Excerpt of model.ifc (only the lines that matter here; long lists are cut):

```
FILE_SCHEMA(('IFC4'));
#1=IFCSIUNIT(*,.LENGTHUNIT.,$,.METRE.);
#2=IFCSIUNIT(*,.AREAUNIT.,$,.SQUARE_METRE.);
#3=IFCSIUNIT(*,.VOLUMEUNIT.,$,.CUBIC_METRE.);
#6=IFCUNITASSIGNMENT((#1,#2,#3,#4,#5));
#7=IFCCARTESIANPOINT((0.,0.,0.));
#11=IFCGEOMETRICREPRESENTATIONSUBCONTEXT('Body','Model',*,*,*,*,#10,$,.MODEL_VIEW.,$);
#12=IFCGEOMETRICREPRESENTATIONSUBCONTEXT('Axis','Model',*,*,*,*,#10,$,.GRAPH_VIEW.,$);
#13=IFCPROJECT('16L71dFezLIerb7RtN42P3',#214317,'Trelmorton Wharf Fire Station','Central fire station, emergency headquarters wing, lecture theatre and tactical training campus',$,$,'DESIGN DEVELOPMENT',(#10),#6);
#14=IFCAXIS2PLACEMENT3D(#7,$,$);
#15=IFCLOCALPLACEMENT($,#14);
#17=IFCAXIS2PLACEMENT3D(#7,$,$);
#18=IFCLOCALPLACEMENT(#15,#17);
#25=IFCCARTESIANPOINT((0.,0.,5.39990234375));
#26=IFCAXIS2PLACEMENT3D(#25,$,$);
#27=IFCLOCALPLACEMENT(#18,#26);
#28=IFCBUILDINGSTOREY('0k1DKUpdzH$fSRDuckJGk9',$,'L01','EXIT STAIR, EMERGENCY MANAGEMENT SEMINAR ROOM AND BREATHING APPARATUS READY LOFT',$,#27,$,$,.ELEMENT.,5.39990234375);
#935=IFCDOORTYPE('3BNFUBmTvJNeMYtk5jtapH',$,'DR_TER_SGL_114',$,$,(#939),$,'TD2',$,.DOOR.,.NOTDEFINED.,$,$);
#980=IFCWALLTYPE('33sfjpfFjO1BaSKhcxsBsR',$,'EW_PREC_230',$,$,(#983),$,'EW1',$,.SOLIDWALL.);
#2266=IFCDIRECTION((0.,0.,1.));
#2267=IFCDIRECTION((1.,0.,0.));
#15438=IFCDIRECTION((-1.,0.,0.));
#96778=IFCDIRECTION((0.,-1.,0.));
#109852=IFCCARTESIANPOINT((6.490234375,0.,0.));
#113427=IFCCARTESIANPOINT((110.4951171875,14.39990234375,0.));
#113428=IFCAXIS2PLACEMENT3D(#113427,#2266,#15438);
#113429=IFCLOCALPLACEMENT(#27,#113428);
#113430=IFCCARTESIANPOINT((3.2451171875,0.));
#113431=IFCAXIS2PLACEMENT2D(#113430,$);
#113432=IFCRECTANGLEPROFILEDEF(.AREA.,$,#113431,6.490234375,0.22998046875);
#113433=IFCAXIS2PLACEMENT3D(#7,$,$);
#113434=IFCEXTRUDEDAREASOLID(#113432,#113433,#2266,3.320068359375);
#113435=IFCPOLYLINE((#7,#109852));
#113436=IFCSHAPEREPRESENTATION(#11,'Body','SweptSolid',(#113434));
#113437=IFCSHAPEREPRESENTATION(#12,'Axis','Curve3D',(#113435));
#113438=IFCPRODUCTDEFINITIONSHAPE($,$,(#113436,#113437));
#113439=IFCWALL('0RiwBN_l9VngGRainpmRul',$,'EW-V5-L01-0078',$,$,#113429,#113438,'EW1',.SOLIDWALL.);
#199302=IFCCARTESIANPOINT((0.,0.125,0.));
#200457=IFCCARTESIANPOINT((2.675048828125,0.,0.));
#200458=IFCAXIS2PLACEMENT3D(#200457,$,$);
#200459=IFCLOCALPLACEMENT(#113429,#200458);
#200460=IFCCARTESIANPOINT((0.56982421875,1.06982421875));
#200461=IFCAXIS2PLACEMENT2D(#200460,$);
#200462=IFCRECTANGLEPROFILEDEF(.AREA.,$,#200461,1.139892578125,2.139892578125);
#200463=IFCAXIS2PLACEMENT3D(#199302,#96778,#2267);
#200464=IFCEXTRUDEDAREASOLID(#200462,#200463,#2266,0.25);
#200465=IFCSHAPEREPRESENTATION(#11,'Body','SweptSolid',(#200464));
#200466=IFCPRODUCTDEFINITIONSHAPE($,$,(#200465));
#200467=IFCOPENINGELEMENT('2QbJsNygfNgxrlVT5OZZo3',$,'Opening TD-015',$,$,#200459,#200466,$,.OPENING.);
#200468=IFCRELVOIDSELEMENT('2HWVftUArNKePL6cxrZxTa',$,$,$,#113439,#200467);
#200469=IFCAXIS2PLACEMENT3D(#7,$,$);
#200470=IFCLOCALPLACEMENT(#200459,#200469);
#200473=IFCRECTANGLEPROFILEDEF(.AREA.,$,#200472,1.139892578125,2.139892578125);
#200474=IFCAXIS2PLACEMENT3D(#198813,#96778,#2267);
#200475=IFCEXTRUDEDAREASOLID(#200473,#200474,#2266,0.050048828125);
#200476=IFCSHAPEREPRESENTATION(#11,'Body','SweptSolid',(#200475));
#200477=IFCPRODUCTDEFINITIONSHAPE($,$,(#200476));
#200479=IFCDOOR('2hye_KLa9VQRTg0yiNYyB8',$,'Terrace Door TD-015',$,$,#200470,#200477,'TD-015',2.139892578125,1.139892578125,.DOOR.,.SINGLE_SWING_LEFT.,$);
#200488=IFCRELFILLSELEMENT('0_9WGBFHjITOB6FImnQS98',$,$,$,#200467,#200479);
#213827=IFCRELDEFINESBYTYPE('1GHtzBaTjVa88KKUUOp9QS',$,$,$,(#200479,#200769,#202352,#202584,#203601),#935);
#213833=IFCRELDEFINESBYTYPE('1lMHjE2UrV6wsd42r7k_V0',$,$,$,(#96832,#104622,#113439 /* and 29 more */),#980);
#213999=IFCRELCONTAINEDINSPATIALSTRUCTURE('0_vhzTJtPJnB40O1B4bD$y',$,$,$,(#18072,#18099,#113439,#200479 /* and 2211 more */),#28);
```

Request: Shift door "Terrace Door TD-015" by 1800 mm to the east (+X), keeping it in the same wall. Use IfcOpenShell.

```python
import ifcopenshell
import ifcopenshell.api.geometry
import ifcopenshell.util.placement
import ifcopenshell.util.unit

model = ifcopenshell.open("model.ifc")
unit_scale = ifcopenshell.util.unit.calculate_unit_scale(model)

door = model.by_guid("2hye_KLa9VQRTg0yiNYyB8")
opening = door.FillsVoids[0].RelatingOpeningElement
wall = opening.VoidsElements[0].RelatingBuildingElement

wall_matrix = ifcopenshell.util.placement.get_local_placement(wall.ObjectPlacement)
shift = wall_matrix[:3, 0] * -1.8 / unit_scale
before = ifcopenshell.util.placement.get_local_placement(door.ObjectPlacement)[:3, 3].copy()

# The door is placed relative to its opening, so it follows when the opening moves.
matrix = ifcopenshell.util.placement.get_local_placement(opening.ObjectPlacement)
matrix[:3, 3] += shift
ifcopenshell.api.geometry.edit_object_placement(
    model, product=opening, matrix=matrix, is_si=False, should_transform_children=True
)

after = ifcopenshell.util.placement.get_local_placement(door.ObjectPlacement)[:3, 3]
print("door moved by", (after - before).round(3) + 0.0)

model.write("model-out.ifc")
```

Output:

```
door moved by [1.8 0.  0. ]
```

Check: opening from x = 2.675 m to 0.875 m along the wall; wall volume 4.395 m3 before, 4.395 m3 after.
